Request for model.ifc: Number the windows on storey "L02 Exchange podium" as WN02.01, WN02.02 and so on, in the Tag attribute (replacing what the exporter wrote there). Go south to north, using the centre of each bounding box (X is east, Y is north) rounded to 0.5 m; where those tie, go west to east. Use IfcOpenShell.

First a look at what the model holds.

```python
import ifcopenshell
import ifcopenshell.util.element
import ifcopenshell.util.placement

model = ifcopenshell.open("model.ifc")
print(model.schema)
storey = next(s for s in model.by_type("IfcBuildingStorey") if s.Name == "L02 Exchange podium")
windows = [e for e in ifcopenshell.util.element.get_decomposition(storey) if e.is_a("IfcWindow")]
for e in sorted(windows, key=lambda e: e.id()):
    origin = ifcopenshell.util.placement.get_local_placement(e.ObjectPlacement)[:3, 3]
    print(e.id(), e.Tag, e.Name, origin.round(2) + 0.0, sep=" | ")
```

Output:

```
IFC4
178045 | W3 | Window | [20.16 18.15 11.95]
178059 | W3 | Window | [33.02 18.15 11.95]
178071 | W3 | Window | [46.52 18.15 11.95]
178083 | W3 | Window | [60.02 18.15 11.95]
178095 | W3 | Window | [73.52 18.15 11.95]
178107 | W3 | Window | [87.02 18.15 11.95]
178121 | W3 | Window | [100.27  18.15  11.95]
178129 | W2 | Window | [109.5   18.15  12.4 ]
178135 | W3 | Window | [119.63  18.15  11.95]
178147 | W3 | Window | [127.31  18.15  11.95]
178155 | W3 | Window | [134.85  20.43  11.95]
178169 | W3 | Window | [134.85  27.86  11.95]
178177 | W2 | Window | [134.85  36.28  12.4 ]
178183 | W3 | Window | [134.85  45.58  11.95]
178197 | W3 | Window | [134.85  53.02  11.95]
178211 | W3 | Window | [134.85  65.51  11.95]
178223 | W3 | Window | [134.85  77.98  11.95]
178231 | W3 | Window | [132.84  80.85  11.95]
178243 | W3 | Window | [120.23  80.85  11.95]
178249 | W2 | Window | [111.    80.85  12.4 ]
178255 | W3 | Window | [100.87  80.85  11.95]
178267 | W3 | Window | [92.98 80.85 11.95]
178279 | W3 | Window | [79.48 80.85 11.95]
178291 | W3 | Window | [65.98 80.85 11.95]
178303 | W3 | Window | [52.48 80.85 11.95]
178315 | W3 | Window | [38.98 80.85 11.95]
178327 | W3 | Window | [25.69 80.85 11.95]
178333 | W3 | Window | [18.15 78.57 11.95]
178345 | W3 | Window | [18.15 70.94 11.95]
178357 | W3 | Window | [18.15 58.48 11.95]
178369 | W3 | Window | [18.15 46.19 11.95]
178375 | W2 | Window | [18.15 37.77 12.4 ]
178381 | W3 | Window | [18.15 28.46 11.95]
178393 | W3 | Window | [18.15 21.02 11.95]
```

```python
import ifcopenshell
import ifcopenshell.geom
import ifcopenshell.util.element
import ifcopenshell.util.shape

model = ifcopenshell.open("model.ifc")
settings = ifcopenshell.geom.settings()
settings.set("use-world-coords", True)


def centre(element):
    shape = ifcopenshell.geom.create_shape(settings, element)
    return ifcopenshell.util.shape.get_bbox_centroid(shape.geometry)


storey = next(s for s in model.by_type("IfcBuildingStorey") if s.Name == "L02 Exchange podium")
windows = [e for e in ifcopenshell.util.element.get_decomposition(storey) if e.is_a("IfcWindow")]

# Insertion points can sit at a corner or the storey origin, so sort by the geometry (in metres).
centres = {e: centre(e) for e in windows}
windows.sort(key=lambda e: (round(centres[e][1] / 0.5), centres[e][0]))

for i, e in enumerate(windows, start=1):
    number = f"WN02.{i:02d}"
    e.Tag = number
    print(e.id(), number)

model.write("model_edited.ifc")
```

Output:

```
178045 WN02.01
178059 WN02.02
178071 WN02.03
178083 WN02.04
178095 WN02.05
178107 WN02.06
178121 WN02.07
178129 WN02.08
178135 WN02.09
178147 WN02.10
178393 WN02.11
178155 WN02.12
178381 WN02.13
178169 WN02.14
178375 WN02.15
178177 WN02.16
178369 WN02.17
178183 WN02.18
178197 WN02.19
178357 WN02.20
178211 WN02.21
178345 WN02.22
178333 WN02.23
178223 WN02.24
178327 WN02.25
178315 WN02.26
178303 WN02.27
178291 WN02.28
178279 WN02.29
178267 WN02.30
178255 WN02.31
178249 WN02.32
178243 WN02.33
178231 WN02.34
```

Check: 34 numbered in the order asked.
